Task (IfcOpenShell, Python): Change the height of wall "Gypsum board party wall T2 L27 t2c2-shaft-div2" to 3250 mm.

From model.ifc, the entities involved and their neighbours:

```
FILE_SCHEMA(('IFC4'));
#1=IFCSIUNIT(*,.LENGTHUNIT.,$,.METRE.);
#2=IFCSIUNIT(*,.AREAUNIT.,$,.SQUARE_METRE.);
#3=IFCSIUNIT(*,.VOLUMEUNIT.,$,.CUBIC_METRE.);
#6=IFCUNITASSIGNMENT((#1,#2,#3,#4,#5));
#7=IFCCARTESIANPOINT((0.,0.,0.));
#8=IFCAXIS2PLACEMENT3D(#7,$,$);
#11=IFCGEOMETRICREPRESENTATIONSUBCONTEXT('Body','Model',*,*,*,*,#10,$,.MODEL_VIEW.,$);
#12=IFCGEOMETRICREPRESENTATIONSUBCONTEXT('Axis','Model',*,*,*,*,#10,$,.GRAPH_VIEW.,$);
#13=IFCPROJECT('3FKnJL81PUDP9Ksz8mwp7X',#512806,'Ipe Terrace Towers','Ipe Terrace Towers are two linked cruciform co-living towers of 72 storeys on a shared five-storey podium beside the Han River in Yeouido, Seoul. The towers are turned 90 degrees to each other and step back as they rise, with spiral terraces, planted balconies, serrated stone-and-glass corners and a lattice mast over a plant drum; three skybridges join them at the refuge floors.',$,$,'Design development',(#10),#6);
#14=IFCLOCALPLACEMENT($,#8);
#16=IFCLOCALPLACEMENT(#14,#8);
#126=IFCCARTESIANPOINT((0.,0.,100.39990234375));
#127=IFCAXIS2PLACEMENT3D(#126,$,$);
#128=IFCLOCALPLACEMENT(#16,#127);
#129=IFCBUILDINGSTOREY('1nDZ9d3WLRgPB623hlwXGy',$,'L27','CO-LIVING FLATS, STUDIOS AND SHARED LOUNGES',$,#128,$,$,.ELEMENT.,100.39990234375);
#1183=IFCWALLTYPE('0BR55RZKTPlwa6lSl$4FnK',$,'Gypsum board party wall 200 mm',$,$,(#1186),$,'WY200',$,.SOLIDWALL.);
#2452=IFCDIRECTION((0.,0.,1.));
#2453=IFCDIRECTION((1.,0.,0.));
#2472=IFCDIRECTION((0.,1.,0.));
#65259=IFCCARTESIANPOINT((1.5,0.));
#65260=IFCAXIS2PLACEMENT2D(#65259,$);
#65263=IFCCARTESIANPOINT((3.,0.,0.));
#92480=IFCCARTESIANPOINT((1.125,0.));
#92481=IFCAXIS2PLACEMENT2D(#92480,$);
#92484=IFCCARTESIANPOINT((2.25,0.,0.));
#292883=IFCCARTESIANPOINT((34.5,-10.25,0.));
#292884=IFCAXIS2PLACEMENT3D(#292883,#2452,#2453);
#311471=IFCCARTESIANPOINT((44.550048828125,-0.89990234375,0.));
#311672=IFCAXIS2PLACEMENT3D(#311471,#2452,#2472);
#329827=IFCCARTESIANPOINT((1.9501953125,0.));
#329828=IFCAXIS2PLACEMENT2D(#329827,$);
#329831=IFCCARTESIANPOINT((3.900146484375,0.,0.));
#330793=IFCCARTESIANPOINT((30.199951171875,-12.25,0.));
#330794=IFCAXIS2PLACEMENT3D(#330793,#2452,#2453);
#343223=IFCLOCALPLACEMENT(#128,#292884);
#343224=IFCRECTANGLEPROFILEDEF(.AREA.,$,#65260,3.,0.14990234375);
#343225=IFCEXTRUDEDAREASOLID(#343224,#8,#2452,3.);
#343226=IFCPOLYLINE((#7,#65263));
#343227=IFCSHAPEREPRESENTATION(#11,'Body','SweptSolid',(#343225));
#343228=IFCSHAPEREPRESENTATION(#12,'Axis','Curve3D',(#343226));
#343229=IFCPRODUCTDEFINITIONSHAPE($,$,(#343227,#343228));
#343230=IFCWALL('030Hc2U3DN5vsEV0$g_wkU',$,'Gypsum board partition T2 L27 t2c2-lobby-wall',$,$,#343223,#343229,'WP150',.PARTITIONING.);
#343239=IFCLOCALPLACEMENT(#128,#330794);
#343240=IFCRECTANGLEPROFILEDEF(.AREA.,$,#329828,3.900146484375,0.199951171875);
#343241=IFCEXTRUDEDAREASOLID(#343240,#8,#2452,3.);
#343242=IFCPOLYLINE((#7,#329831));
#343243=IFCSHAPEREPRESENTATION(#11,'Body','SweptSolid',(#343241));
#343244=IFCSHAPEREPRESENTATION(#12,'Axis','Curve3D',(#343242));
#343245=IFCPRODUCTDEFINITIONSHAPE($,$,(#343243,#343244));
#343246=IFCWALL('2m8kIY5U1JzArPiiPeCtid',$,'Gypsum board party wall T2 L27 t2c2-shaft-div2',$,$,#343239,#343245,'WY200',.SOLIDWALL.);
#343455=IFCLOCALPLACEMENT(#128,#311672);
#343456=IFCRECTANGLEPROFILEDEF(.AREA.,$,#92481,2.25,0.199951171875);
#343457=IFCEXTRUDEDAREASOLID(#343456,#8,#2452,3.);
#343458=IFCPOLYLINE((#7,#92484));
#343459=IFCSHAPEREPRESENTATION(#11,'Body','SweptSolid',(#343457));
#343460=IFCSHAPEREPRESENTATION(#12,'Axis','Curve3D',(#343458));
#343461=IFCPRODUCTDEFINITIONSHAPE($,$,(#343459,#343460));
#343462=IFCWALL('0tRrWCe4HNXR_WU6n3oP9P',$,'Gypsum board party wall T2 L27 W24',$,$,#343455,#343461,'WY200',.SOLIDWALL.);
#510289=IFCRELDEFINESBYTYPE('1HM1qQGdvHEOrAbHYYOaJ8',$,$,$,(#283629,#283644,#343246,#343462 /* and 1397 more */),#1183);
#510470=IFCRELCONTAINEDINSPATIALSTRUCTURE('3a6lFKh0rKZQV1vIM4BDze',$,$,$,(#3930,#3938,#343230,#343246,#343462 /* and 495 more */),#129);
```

```python
import ifcopenshell
import ifcopenshell.geom
import ifcopenshell.util.representation
import ifcopenshell.util.shape
import ifcopenshell.util.unit

model = ifcopenshell.open("model.ifc")
unit_scale = ifcopenshell.util.unit.calculate_unit_scale(model)
settings = ifcopenshell.geom.settings()


def volume(element):
    """Net volume in cubic metres, openings subtracted."""
    shape = ifcopenshell.geom.create_shape(settings, element)
    return ifcopenshell.util.shape.get_volume(shape.geometry)


wall = model.by_id(343246)
before = volume(wall)

body = ifcopenshell.util.representation.get_representation(wall, "Model", "Body")
solid = body.Items[0]
old_height = solid.Depth
solid.Depth = 3.25 / unit_scale
after = volume(wall)

print(f"height {old_height:g} -> {solid.Depth:g}, volume {before:.3f} -> {after:.3f} m3")

model.write("model_updated.ifc")
```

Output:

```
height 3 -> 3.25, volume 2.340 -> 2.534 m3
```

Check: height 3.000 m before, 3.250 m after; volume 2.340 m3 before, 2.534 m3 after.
